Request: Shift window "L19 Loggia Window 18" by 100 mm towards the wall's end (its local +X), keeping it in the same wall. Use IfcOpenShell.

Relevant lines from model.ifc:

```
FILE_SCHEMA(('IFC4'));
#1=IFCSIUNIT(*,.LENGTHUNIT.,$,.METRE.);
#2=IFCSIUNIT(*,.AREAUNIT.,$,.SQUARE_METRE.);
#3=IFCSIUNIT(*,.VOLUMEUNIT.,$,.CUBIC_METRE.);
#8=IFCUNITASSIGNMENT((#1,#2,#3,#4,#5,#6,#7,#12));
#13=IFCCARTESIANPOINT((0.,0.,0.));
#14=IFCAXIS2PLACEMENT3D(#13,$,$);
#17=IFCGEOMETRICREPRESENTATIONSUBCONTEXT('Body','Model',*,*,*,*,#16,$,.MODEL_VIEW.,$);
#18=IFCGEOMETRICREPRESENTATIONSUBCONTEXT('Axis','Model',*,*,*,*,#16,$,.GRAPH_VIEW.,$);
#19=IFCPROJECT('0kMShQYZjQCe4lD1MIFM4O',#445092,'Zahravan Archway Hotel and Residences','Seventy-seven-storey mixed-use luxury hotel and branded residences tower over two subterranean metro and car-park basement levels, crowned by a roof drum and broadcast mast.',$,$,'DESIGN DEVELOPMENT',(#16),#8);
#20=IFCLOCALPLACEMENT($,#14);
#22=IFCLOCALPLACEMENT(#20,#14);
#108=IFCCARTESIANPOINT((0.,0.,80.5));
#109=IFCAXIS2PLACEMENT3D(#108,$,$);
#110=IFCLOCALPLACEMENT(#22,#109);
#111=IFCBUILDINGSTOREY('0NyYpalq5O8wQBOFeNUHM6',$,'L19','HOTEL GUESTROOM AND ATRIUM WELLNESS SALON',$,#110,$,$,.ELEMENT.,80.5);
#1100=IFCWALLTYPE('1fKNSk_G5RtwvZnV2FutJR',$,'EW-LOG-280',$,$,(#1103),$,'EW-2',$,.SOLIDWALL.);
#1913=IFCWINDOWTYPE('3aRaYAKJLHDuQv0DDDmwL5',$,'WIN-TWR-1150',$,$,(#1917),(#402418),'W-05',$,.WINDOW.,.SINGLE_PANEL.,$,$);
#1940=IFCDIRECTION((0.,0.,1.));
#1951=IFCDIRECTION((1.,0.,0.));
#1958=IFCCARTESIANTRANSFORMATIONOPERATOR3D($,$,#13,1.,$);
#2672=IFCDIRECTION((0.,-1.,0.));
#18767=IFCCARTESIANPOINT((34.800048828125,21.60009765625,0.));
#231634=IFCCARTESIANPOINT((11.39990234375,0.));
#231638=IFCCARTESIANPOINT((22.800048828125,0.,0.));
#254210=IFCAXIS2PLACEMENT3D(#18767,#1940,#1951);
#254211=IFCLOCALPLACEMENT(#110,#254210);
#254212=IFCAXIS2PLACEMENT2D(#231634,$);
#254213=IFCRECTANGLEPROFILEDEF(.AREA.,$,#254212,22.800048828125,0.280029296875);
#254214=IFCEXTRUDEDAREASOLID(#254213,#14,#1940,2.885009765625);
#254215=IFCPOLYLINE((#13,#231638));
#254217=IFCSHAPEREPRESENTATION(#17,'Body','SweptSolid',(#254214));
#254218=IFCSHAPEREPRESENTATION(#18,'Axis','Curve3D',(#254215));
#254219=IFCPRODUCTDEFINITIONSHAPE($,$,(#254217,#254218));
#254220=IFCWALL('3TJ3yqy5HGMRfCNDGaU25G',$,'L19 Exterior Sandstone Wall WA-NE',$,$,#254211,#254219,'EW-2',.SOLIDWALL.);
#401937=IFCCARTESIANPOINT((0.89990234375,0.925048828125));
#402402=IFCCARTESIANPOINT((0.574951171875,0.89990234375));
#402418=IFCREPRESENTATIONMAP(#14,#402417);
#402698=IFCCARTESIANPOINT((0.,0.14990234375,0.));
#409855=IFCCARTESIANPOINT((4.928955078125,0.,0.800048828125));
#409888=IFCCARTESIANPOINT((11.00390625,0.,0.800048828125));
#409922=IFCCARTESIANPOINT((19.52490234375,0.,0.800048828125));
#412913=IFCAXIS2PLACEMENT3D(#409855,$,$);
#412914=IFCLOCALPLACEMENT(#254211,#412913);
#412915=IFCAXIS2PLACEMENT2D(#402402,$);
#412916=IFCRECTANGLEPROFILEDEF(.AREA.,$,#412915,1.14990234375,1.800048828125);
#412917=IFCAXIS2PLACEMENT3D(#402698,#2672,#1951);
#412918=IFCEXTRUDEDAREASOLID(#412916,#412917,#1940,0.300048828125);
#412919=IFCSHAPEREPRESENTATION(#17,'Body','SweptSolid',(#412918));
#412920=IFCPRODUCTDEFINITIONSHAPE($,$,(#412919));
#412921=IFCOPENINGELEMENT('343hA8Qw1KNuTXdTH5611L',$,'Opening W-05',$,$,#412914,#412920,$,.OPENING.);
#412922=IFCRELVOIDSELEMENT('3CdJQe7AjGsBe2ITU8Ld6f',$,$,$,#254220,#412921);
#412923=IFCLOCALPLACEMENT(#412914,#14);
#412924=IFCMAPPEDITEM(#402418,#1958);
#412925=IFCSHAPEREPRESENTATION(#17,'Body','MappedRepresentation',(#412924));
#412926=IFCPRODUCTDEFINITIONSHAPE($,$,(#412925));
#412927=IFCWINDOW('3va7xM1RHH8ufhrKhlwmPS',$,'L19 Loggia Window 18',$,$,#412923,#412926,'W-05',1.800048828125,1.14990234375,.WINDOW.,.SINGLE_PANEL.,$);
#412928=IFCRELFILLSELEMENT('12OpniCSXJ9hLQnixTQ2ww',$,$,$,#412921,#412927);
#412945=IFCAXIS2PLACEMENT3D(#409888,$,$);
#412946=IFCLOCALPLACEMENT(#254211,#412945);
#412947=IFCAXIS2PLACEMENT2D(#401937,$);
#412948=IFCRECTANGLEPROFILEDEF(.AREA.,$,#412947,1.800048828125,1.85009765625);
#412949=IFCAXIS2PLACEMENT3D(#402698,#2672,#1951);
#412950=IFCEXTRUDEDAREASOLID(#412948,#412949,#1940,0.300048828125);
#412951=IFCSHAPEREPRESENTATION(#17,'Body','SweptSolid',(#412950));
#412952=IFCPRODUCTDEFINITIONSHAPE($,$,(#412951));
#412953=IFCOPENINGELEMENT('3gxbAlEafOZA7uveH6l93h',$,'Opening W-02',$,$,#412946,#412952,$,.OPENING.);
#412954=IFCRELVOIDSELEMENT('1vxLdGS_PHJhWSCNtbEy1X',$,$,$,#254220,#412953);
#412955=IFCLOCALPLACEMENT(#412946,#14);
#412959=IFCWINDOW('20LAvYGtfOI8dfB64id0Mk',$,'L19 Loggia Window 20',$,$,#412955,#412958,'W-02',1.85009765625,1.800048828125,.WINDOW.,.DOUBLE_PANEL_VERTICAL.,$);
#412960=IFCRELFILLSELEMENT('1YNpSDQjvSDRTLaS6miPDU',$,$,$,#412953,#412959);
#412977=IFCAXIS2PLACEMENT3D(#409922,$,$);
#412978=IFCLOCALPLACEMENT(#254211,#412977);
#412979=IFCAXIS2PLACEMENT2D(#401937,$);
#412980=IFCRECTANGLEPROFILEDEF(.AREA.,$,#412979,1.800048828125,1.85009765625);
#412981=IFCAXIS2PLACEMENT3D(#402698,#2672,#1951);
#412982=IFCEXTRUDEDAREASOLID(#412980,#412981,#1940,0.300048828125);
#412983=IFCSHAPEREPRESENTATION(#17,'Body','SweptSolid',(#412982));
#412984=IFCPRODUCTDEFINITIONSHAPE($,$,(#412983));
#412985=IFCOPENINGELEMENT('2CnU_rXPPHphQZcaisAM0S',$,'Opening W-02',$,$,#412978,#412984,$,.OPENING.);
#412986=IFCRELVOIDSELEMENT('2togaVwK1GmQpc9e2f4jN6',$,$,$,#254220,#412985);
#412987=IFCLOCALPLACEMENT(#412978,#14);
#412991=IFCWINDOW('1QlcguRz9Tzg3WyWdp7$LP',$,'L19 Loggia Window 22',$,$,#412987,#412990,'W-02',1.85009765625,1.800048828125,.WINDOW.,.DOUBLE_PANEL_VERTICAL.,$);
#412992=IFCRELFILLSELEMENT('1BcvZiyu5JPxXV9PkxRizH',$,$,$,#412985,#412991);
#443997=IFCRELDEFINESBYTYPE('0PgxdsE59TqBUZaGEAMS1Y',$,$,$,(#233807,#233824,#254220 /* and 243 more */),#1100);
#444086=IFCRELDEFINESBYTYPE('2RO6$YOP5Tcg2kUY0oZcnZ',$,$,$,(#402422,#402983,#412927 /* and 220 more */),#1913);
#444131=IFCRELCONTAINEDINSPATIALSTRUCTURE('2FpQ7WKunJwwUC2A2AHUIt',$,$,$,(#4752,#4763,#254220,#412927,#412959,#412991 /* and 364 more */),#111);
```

```python
import ifcopenshell
import ifcopenshell.api.geometry
import ifcopenshell.util.placement
import ifcopenshell.util.unit

model = ifcopenshell.open("model.ifc")
unit_scale = ifcopenshell.util.unit.calculate_unit_scale(model)

window = model.by_guid("3va7xM1RHH8ufhrKhlwmPS")
opening = window.FillsVoids[0].RelatingOpeningElement
wall = opening.VoidsElements[0].RelatingBuildingElement

wall_matrix = ifcopenshell.util.placement.get_local_placement(wall.ObjectPlacement)
shift = wall_matrix[:3, 0] * 0.1 / unit_scale
before = ifcopenshell.util.placement.get_local_placement(window.ObjectPlacement)[:3, 3].copy()

# The window is placed relative to its opening, so it follows when the opening moves.
matrix = ifcopenshell.util.placement.get_local_placement(opening.ObjectPlacement)
matrix[:3, 3] += shift
ifcopenshell.api.geometry.edit_object_placement(
    model, product=opening, matrix=matrix, is_si=False, should_transform_children=True
)

after = ifcopenshell.util.placement.get_local_placement(window.ObjectPlacement)[:3, 3]
print("window moved by", (after - before).round(3) + 0.0)

model.write("model_v2.ifc")
```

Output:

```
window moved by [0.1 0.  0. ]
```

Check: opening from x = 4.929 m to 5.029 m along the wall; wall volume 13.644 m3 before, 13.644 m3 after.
